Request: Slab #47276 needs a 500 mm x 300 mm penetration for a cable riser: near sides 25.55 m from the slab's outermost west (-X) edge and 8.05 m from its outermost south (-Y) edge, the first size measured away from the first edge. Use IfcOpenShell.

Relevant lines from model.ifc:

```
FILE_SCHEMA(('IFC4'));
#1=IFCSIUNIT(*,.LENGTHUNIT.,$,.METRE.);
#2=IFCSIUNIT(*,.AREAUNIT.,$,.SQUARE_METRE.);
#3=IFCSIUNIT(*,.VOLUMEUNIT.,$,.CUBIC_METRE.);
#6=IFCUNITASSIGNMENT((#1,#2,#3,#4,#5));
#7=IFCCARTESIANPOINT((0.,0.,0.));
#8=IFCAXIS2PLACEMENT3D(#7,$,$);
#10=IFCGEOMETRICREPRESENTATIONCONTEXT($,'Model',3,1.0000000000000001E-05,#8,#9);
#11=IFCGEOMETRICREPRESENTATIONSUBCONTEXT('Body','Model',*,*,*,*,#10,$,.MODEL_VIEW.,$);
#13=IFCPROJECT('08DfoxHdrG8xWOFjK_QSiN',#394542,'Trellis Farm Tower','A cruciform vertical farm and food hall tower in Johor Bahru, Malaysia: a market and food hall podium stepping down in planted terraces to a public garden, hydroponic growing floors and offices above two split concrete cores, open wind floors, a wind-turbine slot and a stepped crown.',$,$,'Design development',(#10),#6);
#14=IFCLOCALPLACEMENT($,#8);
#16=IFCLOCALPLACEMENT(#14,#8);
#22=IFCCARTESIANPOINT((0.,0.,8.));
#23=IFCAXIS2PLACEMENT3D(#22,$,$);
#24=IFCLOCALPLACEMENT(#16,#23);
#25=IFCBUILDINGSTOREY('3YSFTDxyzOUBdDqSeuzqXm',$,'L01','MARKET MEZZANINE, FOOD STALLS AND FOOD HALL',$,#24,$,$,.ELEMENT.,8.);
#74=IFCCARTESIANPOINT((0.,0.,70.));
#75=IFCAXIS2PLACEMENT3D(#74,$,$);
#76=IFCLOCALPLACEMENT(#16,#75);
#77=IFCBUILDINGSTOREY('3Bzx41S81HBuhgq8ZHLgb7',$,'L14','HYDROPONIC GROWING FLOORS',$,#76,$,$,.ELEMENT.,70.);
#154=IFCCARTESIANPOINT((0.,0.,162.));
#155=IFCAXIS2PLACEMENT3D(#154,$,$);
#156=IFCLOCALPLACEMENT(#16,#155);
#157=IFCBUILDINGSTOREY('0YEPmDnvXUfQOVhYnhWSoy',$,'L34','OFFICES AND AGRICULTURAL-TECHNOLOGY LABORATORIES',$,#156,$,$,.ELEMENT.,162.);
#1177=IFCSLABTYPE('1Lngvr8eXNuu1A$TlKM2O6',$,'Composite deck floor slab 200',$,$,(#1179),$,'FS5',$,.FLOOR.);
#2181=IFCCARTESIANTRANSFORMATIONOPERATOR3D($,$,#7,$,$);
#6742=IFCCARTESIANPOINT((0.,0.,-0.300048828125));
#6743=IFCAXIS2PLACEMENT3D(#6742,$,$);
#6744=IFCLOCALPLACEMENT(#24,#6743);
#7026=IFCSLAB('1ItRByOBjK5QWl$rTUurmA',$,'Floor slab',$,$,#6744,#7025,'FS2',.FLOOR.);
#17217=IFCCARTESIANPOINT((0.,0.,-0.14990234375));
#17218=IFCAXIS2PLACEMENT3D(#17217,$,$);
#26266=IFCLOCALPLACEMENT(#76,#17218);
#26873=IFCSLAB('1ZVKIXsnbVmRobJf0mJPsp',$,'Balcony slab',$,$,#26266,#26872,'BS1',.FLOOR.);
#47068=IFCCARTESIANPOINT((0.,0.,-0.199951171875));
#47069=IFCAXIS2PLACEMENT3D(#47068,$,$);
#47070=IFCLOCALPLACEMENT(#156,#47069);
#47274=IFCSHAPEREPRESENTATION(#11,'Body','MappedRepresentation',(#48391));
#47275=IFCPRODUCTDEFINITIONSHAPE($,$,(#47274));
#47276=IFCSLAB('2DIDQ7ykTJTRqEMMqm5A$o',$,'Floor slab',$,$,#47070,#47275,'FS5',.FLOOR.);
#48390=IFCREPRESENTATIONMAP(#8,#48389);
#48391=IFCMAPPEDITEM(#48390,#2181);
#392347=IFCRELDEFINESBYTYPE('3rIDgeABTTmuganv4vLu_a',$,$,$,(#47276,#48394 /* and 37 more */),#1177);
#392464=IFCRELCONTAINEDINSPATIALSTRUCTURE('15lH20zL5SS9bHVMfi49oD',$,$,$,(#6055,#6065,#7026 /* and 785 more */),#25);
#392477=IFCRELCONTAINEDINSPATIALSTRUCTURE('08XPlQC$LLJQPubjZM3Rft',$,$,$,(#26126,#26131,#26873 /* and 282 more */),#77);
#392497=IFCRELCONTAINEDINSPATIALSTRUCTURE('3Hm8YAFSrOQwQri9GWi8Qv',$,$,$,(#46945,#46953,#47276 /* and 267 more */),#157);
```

```python
import numpy as np
import ifcopenshell
import ifcopenshell.api.feature
import ifcopenshell.api.geometry
import ifcopenshell.api.root
import ifcopenshell.geom
import ifcopenshell.util.placement
import ifcopenshell.util.representation
import ifcopenshell.util.shape
import ifcopenshell.util.unit

model = ifcopenshell.open("model.ifc")
unit_scale = ifcopenshell.util.unit.calculate_unit_scale(model)
settings = ifcopenshell.geom.settings()


def volume(element):
    """Net volume in cubic metres, openings subtracted."""
    shape = ifcopenshell.geom.create_shape(settings, element)
    return ifcopenshell.util.shape.get_volume(shape.geometry)


slab = model.by_id(47276)
before = volume(slab)

# Extent in the slab's own axes, in metres. The edges named are its -X and -Y sides.
slab_shape = ifcopenshell.geom.create_shape(settings, slab)
vertices = ifcopenshell.util.shape.get_vertices(slab_shape.geometry)
x_min, y_min, bottom = vertices.min(axis=0)
top = vertices[:, 2].max()

opening = ifcopenshell.api.root.create_entity(model, ifc_class="IfcOpeningElement", name="Cable riser opening", predefined_type="OPENING")
context = ifcopenshell.util.representation.get_context(model, "Model", "Body", "MODEL_VIEW")
width, depth = 0.5, 0.3
outline = [(0.0, 0.0), (width, 0.0), (width, depth), (0.0, depth), (0.0, 0.0)]
# Overshoot both faces by 50 mm so the cut is clean.
shape = ifcopenshell.api.geometry.add_slab_representation(
    model, context=context, depth=top - bottom + 0.1, polyline=outline
)
ifcopenshell.api.geometry.assign_representation(model, product=opening, representation=shape)

matrix = ifcopenshell.util.placement.get_local_placement(slab.ObjectPlacement)
matrix[:, 3] = matrix @ np.append(np.array([x_min + 25.55, y_min + 8.05, bottom - 0.05]) / unit_scale, 1.0)
ifcopenshell.api.geometry.edit_object_placement(model, product=opening, matrix=matrix, is_si=False)
ifcopenshell.api.feature.add_feature(model, feature=opening, element=slab)

after = volume(slab)

print(f"slab volume {before:.3f} -> {after:.3f} m3")

model.write("model_v2.ifc")
```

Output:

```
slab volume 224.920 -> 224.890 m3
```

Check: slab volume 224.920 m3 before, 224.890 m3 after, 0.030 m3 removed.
